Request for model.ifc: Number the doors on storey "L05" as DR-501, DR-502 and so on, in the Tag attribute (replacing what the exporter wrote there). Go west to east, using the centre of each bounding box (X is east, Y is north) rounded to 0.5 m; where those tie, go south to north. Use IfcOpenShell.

First a look at what the model holds.

```python
import ifcopenshell
import ifcopenshell.util.element
import ifcopenshell.util.placement

model = ifcopenshell.open("model.ifc")
print(model.schema)
storey = next(s for s in model.by_type("IfcBuildingStorey") if s.Name == "L05")
doors = [e for e in ifcopenshell.util.element.get_decomposition(storey) if e.is_a("IfcDoor")]
for e in sorted(doors, key=lambda e: e.id()):
    origin = ifcopenshell.util.placement.get_local_placement(e.ObjectPlacement)[:3, 3]
    print(e.id(), e.Tag, e.Name, origin.round(2) + 0.0, sep=" | ")
```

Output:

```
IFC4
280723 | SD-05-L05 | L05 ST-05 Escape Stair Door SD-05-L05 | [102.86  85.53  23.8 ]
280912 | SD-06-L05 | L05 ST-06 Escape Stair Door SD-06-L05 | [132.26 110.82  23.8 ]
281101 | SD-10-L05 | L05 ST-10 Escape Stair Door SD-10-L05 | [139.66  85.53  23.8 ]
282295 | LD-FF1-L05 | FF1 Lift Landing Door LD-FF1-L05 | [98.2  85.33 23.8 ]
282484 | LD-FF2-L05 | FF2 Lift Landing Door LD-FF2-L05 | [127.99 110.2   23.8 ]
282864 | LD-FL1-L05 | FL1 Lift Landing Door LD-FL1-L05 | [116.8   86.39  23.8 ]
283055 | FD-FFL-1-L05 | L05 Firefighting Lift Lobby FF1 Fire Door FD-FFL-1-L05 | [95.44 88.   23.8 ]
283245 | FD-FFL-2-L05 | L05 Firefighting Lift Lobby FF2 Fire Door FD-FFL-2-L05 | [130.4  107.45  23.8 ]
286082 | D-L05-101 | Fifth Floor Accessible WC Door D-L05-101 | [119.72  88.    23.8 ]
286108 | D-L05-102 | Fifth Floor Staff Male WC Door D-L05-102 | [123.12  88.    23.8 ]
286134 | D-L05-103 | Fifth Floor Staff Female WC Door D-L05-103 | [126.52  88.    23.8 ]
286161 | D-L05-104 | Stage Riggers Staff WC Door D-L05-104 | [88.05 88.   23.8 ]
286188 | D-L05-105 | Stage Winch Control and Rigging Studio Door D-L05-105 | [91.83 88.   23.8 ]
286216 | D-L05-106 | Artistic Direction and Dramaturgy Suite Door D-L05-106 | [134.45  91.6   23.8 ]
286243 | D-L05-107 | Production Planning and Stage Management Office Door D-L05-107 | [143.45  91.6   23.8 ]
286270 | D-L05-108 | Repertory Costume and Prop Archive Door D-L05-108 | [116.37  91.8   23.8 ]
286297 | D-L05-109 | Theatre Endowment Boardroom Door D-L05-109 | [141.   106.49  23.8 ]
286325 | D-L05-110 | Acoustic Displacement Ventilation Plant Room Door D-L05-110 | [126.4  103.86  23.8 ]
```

```python
import ifcopenshell
import ifcopenshell.geom
import ifcopenshell.util.element
import ifcopenshell.util.shape

model = ifcopenshell.open("model.ifc")
settings = ifcopenshell.geom.settings()
settings.set("use-world-coords", True)


def centre(element):
    shape = ifcopenshell.geom.create_shape(settings, element)
    return ifcopenshell.util.shape.get_bbox_centroid(shape.geometry)


storey = next(s for s in model.by_type("IfcBuildingStorey") if s.Name == "L05")
doors = [e for e in ifcopenshell.util.element.get_decomposition(storey) if e.is_a("IfcDoor")]

# Insertion points can sit at a corner or the storey origin, so sort by the geometry (in metres).
centres = {e: centre(e) for e in doors}
doors.sort(key=lambda e: (round(centres[e][0] / 0.5), centres[e][1]))

for i, e in enumerate(doors, start=1):
    number = f"DR-5{i:02d}"
    e.Tag = number
    print(e.id(), number)

model.write("model_updated.ifc")
```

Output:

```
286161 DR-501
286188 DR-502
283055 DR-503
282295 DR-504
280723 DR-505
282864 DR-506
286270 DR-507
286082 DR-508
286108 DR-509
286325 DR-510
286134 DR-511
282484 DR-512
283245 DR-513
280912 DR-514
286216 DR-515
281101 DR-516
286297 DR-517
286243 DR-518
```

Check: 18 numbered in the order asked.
